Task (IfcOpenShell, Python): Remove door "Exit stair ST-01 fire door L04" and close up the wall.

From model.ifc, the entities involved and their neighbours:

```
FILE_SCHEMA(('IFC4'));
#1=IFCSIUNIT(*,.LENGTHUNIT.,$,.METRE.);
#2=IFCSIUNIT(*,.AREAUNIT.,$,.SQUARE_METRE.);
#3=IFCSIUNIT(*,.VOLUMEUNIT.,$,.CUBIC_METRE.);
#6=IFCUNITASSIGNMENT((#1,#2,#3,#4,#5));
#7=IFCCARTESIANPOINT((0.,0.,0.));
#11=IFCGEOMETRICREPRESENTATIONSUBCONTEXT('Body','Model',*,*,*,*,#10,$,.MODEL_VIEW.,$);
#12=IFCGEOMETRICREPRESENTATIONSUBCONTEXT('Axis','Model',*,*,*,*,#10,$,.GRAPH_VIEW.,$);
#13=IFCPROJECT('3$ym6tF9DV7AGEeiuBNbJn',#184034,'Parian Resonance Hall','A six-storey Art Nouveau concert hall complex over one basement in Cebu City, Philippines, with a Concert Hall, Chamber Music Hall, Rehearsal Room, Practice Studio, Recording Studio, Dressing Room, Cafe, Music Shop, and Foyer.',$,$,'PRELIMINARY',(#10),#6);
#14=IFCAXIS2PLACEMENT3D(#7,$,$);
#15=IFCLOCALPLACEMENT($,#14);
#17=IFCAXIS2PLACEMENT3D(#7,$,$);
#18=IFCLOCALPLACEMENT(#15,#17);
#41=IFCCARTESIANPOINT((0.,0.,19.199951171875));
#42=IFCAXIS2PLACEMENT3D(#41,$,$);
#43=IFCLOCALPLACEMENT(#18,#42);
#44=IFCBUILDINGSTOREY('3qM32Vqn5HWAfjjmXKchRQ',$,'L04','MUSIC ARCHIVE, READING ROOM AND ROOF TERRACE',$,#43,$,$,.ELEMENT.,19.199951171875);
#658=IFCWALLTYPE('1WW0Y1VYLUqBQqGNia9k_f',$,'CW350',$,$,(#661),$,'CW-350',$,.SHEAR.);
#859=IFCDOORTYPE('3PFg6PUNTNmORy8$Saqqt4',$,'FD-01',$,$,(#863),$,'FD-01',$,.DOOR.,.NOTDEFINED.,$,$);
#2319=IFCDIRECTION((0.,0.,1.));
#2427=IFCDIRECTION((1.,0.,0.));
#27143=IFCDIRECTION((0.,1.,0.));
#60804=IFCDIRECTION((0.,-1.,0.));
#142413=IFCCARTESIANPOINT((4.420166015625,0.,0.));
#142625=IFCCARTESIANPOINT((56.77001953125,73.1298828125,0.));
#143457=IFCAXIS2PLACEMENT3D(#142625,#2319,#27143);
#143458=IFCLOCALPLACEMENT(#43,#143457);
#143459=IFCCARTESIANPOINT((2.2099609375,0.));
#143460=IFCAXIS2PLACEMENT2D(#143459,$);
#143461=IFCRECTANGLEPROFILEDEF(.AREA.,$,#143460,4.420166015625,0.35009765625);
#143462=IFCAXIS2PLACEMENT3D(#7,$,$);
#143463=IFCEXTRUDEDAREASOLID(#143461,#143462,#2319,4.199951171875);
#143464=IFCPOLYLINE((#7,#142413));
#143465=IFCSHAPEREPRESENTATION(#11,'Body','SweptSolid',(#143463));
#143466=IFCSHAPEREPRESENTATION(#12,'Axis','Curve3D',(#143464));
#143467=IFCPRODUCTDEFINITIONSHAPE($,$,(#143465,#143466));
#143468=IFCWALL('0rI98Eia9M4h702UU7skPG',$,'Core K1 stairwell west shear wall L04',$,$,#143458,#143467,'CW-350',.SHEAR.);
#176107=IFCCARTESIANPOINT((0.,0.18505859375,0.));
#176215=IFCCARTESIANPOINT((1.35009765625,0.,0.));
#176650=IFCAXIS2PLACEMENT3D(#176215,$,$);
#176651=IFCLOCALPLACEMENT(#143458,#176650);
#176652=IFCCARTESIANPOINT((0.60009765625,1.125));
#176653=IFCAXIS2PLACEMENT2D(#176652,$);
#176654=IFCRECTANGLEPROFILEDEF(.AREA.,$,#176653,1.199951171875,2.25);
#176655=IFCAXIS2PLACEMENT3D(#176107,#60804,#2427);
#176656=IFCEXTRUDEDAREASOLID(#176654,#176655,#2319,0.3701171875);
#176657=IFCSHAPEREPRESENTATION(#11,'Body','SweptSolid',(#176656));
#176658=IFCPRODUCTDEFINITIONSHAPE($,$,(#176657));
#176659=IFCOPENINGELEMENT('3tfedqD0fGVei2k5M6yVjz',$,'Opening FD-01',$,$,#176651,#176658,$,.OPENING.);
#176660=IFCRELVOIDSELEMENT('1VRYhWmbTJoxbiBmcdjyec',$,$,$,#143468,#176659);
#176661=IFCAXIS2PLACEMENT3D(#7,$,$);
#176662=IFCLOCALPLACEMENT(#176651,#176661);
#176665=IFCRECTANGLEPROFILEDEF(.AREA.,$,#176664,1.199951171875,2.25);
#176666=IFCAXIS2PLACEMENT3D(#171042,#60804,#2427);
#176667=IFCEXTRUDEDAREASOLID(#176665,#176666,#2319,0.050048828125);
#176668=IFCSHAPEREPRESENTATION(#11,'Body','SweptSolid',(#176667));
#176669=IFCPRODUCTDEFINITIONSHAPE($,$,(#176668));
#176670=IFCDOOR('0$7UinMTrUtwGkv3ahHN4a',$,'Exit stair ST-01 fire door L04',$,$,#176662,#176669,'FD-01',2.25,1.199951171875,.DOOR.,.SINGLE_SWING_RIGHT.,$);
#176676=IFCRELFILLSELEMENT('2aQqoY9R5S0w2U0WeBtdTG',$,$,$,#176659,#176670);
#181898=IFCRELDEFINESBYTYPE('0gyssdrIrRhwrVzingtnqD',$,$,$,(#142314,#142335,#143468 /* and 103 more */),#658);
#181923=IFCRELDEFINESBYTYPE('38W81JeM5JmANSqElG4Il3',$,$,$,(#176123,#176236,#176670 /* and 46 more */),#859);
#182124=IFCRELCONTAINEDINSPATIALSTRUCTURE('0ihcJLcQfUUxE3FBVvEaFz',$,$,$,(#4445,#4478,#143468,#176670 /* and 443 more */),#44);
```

```python
import ifcopenshell
import ifcopenshell.api.feature
import ifcopenshell.api.root
import ifcopenshell.geom
import ifcopenshell.util.shape

model = ifcopenshell.open("model.ifc")
settings = ifcopenshell.geom.settings()


def volume(element):
    """Net volume in cubic metres, openings subtracted."""
    shape = ifcopenshell.geom.create_shape(settings, element)
    return ifcopenshell.util.shape.get_volume(shape.geometry)


door = model.by_guid("0$7UinMTrUtwGkv3ahHN4a")
opening = door.FillsVoids[0].RelatingOpeningElement
wall = opening.VoidsElements[0].RelatingBuildingElement
before = volume(wall)

ifcopenshell.api.root.remove_product(model, product=door)
ifcopenshell.api.feature.remove_feature(model, feature=opening)

after = volume(wall)

print(f"wall volume {before:.3f} -> {after:.3f} m3")

model.write("model_edited.ifc")
```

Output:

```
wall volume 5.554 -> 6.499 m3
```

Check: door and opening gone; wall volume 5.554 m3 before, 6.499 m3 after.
